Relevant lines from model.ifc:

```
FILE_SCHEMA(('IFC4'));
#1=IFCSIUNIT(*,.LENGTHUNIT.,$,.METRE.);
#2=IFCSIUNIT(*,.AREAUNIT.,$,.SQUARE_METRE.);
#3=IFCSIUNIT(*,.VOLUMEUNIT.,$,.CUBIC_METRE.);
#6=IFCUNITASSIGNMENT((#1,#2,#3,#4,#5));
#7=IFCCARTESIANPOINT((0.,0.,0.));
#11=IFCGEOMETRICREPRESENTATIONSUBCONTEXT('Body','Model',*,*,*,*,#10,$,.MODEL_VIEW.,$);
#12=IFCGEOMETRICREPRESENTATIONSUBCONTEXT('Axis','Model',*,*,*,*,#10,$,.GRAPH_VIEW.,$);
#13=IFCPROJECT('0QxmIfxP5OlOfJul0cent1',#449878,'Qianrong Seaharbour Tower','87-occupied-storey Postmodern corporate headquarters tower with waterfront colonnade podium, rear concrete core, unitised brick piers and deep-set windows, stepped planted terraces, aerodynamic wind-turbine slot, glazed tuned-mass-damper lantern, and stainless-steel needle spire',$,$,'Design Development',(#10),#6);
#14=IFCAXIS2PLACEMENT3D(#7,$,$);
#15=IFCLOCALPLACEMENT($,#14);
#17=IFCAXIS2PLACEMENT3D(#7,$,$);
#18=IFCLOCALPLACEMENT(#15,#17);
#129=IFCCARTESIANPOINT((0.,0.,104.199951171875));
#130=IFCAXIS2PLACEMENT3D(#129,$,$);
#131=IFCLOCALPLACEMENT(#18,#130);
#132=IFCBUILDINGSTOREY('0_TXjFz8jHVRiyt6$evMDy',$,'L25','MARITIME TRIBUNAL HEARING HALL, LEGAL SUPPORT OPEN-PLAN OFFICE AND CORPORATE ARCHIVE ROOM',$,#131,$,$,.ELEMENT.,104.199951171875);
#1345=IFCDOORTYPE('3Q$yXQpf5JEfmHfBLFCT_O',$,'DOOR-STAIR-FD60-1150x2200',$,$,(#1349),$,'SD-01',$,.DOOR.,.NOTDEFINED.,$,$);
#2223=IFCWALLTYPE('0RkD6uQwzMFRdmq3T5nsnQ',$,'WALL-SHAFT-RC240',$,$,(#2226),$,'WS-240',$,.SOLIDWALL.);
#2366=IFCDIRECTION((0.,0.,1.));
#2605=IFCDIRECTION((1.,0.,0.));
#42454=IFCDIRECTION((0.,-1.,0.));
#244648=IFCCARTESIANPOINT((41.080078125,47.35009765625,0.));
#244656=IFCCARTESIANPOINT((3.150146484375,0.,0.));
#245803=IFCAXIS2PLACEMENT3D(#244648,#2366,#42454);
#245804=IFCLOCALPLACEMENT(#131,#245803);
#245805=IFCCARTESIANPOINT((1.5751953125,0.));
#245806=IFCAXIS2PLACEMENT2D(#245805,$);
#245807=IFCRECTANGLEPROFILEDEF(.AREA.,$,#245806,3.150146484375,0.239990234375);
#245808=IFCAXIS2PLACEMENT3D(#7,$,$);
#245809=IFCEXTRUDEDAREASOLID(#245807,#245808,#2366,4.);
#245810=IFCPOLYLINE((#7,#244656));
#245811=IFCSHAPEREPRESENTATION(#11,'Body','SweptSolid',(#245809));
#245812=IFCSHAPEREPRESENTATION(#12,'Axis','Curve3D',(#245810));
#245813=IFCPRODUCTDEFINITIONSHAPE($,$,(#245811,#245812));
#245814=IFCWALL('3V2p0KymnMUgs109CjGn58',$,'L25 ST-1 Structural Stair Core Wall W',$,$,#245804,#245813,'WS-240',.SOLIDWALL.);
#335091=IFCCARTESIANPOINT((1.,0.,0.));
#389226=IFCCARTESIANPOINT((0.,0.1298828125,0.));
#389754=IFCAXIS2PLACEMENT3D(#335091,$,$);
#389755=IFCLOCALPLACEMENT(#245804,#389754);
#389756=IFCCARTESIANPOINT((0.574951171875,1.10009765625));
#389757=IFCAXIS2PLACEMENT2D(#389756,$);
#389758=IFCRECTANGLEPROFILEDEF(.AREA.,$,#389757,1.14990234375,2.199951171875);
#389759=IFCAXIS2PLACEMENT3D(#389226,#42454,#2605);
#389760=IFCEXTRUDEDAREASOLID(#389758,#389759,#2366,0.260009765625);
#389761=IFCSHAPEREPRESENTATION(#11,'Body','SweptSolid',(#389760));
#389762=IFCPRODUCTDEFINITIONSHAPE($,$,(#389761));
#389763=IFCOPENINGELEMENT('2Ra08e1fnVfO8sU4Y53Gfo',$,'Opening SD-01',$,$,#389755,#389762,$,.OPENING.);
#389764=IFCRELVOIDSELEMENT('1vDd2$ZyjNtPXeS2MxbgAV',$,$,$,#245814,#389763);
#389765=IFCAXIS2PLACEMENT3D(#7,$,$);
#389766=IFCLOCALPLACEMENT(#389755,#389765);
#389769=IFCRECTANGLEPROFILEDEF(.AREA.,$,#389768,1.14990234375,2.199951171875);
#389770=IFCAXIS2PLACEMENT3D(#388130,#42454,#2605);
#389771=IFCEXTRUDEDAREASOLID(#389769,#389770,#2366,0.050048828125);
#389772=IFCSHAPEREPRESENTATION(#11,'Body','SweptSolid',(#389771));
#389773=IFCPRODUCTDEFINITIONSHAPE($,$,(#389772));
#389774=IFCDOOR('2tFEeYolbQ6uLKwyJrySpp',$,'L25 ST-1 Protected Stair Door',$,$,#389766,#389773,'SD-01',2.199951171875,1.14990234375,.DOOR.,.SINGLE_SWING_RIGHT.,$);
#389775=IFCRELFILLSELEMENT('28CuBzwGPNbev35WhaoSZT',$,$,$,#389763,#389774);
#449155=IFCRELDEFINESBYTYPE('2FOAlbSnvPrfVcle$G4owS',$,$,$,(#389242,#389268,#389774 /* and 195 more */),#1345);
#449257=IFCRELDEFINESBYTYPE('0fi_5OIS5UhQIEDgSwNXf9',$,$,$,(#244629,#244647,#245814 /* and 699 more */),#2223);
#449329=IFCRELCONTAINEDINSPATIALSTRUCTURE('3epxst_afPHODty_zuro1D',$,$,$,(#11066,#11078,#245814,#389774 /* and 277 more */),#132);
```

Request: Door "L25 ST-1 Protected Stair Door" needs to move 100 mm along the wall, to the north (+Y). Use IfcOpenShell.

```python
import ifcopenshell
import ifcopenshell.api.geometry
import ifcopenshell.util.placement

model = ifcopenshell.open("model.ifc")

door = model.by_id(389774)
opening = door.FillsVoids[0].RelatingOpeningElement
wall = opening.VoidsElements[0].RelatingBuildingElement

wall_matrix = ifcopenshell.util.placement.get_local_placement(wall.ObjectPlacement)
shift = wall_matrix[:3, 0] * -0.1
before = ifcopenshell.util.placement.get_local_placement(door.ObjectPlacement)[:3, 3].copy()

# The door is placed relative to its opening, so it follows when the opening moves.
matrix = ifcopenshell.util.placement.get_local_placement(opening.ObjectPlacement)
matrix[:3, 3] += shift
ifcopenshell.api.geometry.edit_object_placement(
    model, product=opening, matrix=matrix, is_si=False, should_transform_children=True
)

after = ifcopenshell.util.placement.get_local_placement(door.ObjectPlacement)[:3, 3]
print("door moved by", (after - before).round(3) + 0.0)

model.write("model_updated.ifc")
```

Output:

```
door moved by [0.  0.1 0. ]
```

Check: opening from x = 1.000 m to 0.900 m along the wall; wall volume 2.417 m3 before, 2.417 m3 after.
